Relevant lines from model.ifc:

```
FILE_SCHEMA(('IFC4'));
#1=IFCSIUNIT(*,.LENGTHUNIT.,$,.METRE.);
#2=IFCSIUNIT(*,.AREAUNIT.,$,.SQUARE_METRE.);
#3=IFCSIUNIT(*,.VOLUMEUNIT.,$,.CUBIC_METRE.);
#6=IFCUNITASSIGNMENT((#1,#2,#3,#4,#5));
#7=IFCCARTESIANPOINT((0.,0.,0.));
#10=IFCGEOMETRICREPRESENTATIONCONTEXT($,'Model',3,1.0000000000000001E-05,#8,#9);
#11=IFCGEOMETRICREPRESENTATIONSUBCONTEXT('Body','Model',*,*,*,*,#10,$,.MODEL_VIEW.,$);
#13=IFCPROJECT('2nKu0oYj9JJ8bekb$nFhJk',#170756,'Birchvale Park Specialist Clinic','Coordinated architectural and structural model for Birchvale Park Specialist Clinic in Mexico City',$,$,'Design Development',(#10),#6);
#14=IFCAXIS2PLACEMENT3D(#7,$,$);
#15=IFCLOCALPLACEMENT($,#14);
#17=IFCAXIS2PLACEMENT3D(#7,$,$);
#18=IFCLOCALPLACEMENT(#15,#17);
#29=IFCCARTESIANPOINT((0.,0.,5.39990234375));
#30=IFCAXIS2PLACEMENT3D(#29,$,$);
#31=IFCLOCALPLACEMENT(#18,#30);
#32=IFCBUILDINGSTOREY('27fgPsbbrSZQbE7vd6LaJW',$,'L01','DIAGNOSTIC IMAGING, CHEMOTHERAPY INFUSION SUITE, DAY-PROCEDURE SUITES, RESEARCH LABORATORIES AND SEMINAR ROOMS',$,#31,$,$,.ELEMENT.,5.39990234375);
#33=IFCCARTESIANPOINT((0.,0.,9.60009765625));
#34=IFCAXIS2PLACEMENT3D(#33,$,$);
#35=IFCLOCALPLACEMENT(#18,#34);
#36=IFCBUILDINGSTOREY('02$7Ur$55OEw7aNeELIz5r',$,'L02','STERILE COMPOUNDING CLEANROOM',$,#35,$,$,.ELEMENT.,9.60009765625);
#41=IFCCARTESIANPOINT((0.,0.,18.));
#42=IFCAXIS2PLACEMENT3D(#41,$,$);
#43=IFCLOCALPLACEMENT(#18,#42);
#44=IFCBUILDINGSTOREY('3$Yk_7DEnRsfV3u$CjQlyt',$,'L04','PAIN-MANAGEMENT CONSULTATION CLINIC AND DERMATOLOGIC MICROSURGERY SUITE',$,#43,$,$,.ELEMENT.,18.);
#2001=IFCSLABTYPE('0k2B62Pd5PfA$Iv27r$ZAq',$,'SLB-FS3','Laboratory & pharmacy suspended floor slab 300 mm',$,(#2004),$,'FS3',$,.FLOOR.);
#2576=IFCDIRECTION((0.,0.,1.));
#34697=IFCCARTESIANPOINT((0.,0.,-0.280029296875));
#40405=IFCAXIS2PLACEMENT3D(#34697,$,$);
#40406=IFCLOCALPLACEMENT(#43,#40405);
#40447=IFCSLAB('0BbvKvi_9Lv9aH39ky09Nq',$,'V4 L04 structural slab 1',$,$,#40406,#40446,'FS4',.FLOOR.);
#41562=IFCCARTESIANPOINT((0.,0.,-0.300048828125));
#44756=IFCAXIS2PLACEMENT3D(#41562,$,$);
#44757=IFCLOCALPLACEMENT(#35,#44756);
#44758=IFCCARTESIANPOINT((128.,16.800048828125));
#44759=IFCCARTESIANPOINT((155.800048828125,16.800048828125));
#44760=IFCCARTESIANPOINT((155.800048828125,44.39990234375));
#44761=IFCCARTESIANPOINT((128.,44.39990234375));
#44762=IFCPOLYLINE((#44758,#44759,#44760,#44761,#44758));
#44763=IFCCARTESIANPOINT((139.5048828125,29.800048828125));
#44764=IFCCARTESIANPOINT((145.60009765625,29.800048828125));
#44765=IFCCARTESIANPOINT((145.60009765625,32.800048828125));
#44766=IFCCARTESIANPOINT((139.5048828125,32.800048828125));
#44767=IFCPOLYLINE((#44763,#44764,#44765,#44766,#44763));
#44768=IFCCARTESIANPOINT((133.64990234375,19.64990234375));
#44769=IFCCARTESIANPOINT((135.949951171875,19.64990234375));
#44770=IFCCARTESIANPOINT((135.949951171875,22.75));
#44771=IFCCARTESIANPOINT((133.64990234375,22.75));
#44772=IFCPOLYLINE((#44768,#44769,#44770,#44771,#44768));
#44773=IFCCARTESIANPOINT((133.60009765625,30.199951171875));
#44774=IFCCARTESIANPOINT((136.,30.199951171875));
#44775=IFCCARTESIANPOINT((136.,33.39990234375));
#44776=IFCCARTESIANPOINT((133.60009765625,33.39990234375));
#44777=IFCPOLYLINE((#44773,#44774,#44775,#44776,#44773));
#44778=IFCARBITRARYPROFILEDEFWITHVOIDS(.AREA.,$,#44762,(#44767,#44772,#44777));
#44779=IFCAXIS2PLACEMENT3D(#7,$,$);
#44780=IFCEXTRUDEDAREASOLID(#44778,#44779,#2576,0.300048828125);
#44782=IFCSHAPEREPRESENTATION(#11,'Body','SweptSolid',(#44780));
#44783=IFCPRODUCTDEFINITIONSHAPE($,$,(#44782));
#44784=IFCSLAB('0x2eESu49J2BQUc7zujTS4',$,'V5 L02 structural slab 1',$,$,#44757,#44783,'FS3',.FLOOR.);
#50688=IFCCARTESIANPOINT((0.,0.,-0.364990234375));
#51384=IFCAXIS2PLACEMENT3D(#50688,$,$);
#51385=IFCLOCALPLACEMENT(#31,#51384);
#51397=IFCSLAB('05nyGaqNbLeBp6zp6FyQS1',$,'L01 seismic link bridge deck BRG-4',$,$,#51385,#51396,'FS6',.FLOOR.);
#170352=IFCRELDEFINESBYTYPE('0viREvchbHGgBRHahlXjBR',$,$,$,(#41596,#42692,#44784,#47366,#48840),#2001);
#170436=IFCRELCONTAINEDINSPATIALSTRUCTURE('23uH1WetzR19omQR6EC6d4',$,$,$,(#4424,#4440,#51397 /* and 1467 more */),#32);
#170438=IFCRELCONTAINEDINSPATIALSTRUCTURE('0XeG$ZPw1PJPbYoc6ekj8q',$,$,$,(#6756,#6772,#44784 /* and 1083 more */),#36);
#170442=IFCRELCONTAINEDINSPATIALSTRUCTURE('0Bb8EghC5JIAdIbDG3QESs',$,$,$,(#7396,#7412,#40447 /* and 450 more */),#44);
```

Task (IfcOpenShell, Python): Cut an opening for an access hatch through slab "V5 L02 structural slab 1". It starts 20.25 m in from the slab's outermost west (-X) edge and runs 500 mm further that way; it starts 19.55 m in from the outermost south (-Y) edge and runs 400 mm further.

```python
import numpy as np
import ifcopenshell
import ifcopenshell.api.feature
import ifcopenshell.api.geometry
import ifcopenshell.api.root
import ifcopenshell.geom
import ifcopenshell.util.placement
import ifcopenshell.util.representation
import ifcopenshell.util.shape
import ifcopenshell.util.unit

model = ifcopenshell.open("model.ifc")
unit_scale = ifcopenshell.util.unit.calculate_unit_scale(model)
settings = ifcopenshell.geom.settings()


def volume(element):
    """Net volume in cubic metres, openings subtracted."""
    shape = ifcopenshell.geom.create_shape(settings, element)
    return ifcopenshell.util.shape.get_volume(shape.geometry)


slab = model.by_guid("0x2eESu49J2BQUc7zujTS4")
before = volume(slab)

# Extent in the slab's own axes, in metres. The edges named are its -X and -Y sides.
slab_shape = ifcopenshell.geom.create_shape(settings, slab)
vertices = ifcopenshell.util.shape.get_vertices(slab_shape.geometry)
x_min, y_min, bottom = vertices.min(axis=0)
top = vertices[:, 2].max()

opening = ifcopenshell.api.root.create_entity(model, ifc_class="IfcOpeningElement", name="Access hatch opening", predefined_type="OPENING")
context = ifcopenshell.util.representation.get_context(model, "Model", "Body", "MODEL_VIEW")
width, depth = 0.5, 0.4
outline = [(0.0, 0.0), (width, 0.0), (width, depth), (0.0, depth), (0.0, 0.0)]
# Overshoot both faces by 50 mm so the cut is clean.
shape = ifcopenshell.api.geometry.add_slab_representation(
    model, context=context, depth=top - bottom + 0.1, polyline=outline
)
ifcopenshell.api.geometry.assign_representation(model, product=opening, representation=shape)

matrix = ifcopenshell.util.placement.get_local_placement(slab.ObjectPlacement)
matrix[:, 3] = matrix @ np.append(np.array([x_min + 20.25, y_min + 19.55, bottom - 0.05]) / unit_scale, 1.0)
ifcopenshell.api.geometry.edit_object_placement(model, product=opening, matrix=matrix, is_si=False)
ifcopenshell.api.feature.add_feature(model, feature=opening, element=slab)

after = volume(slab)

print(f"slab volume {before:.3f} -> {after:.3f} m3")

model.write("model_edited.ifc")
```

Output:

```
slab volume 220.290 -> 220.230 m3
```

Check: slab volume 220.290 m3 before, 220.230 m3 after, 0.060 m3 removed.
